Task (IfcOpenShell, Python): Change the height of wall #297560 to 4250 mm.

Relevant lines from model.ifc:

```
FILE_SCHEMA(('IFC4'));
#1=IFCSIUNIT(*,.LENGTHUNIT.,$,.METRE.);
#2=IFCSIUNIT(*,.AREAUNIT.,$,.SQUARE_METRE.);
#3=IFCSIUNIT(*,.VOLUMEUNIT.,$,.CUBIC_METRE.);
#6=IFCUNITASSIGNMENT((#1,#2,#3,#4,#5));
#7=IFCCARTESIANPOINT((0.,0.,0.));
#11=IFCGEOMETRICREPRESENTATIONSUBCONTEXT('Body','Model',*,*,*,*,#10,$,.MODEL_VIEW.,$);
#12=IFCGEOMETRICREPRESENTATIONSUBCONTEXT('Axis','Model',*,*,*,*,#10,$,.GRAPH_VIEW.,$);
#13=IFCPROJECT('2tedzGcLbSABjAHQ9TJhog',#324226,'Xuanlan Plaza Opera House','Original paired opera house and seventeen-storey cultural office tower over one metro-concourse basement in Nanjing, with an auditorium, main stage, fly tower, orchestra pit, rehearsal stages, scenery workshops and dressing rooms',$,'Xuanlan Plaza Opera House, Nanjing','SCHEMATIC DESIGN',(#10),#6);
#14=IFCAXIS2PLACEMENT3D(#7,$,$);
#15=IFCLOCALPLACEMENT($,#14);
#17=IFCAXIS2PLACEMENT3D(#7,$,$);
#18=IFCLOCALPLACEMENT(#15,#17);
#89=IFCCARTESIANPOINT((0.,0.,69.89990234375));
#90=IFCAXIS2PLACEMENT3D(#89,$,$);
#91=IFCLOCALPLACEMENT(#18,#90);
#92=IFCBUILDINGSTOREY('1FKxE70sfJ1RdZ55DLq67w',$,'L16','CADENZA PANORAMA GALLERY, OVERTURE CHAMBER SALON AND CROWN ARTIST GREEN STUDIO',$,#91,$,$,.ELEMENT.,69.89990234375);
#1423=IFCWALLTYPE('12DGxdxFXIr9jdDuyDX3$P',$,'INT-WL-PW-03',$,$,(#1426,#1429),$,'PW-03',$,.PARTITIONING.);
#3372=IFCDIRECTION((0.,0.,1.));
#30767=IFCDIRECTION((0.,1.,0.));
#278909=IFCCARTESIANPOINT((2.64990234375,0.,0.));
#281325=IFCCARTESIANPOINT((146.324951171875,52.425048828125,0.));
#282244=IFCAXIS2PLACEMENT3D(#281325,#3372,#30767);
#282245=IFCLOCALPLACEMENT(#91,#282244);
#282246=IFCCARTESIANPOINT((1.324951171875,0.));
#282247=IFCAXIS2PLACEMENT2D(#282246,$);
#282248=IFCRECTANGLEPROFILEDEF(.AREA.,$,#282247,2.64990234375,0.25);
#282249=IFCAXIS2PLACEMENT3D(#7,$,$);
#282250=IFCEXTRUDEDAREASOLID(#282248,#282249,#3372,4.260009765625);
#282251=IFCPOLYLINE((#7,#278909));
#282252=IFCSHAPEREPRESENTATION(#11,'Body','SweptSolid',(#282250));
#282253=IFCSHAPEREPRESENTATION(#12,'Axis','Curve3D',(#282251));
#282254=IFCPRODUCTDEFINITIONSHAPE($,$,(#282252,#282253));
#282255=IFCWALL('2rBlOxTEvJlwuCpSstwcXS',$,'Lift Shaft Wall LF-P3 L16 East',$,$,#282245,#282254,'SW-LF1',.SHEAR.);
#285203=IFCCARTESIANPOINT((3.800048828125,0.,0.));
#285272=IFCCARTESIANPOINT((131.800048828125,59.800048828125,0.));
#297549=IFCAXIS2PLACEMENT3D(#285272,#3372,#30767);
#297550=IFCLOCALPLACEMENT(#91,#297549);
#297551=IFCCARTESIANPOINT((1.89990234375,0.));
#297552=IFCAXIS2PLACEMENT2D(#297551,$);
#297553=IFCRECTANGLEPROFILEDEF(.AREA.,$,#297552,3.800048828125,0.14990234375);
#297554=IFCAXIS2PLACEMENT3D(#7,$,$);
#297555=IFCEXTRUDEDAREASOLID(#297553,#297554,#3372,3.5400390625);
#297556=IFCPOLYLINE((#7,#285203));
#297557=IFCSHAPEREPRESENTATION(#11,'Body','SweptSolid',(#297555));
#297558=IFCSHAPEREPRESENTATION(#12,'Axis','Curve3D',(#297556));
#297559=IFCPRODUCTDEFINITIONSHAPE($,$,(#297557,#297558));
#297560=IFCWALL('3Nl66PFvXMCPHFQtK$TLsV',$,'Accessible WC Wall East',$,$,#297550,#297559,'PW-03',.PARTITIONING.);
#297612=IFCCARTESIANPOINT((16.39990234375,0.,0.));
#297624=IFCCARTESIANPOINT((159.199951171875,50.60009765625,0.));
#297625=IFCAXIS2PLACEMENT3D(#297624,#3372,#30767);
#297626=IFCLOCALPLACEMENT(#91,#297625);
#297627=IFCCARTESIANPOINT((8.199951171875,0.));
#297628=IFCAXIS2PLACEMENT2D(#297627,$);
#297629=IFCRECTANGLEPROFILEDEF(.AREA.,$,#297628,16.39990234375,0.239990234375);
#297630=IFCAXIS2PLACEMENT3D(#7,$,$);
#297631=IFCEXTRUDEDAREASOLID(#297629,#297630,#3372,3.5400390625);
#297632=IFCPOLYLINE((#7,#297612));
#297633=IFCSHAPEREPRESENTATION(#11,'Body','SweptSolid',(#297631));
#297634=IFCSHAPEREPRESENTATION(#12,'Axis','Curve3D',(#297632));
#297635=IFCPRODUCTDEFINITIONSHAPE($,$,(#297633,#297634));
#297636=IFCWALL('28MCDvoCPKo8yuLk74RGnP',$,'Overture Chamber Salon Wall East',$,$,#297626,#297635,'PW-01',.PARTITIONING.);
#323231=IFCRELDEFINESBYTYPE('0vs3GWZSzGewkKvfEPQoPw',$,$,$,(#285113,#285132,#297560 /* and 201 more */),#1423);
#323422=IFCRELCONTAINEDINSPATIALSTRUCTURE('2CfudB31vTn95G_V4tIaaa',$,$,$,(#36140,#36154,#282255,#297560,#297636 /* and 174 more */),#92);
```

```python
import ifcopenshell
import ifcopenshell.geom
import ifcopenshell.util.representation
import ifcopenshell.util.shape

model = ifcopenshell.open("model.ifc")
settings = ifcopenshell.geom.settings()


def volume(element):
    """Net volume in cubic metres, openings subtracted."""
    shape = ifcopenshell.geom.create_shape(settings, element)
    return ifcopenshell.util.shape.get_volume(shape.geometry)


wall = model.by_guid("3Nl66PFvXMCPHFQtK$TLsV")
before = volume(wall)

body = ifcopenshell.util.representation.get_representation(wall, "Model", "Body")
solid = body.Items[0]
old_height = solid.Depth
solid.Depth = 4.25
after = volume(wall)

print(f"height {old_height:g} -> {solid.Depth:g}, volume {before:.3f} -> {after:.3f} m3")

model.write("model_updated.ifc")
```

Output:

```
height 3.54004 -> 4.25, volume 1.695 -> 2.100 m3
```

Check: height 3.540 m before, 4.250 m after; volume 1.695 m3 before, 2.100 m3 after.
